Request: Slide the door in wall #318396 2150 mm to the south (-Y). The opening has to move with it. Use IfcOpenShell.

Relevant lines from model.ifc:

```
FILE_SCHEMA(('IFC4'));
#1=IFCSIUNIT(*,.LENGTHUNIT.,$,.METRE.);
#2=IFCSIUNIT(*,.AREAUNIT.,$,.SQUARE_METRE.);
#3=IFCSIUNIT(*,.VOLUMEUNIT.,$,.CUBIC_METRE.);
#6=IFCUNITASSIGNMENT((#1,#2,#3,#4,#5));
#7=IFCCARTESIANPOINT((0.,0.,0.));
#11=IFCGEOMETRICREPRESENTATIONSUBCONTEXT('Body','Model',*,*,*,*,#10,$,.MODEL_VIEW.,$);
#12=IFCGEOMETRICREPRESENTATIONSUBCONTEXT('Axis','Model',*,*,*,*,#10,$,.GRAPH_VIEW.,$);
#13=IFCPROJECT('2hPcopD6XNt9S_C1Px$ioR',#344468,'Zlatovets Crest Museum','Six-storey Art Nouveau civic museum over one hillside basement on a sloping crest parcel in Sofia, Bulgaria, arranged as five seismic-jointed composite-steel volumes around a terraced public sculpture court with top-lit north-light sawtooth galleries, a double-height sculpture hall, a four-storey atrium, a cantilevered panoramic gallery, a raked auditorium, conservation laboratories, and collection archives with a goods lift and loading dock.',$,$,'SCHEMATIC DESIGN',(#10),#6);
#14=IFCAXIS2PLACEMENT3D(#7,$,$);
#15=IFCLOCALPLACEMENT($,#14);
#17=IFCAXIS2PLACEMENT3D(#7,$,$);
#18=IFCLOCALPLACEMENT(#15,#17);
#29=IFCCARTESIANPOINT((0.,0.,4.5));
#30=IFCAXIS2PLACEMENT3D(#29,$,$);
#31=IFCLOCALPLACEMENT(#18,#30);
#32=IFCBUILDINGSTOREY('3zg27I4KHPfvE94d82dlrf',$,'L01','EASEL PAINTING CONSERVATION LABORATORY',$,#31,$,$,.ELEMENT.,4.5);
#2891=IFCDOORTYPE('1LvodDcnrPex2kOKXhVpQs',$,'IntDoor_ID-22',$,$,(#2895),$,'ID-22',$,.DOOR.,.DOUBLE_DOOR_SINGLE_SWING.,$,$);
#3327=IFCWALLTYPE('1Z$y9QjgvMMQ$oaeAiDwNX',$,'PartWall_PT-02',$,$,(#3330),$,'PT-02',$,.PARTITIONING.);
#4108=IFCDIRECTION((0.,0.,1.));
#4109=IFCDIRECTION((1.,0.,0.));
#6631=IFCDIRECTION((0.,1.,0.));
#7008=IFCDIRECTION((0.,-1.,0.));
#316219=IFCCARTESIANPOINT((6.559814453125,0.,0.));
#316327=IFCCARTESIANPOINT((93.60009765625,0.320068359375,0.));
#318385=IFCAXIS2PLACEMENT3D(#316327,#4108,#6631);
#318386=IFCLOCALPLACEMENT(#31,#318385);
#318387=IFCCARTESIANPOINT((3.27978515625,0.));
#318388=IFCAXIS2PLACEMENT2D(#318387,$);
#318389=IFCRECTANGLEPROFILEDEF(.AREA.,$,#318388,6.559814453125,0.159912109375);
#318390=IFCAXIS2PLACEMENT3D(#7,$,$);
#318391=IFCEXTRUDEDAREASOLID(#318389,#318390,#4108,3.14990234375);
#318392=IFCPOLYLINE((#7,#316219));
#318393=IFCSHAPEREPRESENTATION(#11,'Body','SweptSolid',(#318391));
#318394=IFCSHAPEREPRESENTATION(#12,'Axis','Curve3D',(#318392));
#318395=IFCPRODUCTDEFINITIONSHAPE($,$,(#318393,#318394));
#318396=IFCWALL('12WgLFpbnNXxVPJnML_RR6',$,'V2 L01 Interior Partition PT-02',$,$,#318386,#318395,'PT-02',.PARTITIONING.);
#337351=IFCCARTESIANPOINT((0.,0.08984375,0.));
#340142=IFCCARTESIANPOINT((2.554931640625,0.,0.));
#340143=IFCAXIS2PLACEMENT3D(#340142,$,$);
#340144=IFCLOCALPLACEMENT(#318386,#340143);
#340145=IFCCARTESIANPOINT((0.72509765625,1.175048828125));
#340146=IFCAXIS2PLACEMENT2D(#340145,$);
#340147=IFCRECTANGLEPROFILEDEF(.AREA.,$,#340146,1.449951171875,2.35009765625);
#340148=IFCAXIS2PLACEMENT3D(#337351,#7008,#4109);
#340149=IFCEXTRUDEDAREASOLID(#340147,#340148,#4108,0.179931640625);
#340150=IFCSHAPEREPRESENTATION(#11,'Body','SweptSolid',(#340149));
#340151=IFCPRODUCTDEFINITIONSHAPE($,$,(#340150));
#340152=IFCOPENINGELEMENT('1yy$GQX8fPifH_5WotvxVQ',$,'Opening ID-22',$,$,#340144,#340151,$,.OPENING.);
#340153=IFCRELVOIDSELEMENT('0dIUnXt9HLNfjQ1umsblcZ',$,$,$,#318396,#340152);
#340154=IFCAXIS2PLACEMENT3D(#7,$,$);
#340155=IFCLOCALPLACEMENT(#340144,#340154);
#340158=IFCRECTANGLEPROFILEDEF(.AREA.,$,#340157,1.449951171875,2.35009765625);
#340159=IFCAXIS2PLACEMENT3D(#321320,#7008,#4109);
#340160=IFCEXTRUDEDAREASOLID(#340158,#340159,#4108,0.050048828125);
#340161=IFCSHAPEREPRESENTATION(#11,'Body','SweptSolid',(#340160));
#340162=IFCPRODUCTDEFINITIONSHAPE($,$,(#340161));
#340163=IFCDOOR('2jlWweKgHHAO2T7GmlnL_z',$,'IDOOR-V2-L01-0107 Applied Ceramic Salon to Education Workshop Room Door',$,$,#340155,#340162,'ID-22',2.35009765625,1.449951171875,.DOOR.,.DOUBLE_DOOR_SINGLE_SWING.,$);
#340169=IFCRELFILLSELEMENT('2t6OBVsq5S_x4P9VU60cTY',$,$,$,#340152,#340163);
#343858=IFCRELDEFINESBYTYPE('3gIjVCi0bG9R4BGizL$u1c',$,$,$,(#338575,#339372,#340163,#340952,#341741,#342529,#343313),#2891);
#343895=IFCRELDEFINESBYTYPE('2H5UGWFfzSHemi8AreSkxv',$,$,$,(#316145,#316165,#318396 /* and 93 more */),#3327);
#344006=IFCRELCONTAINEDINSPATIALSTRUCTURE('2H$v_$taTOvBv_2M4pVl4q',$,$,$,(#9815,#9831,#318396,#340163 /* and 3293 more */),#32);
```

```python
import ifcopenshell
import ifcopenshell.api.geometry
import ifcopenshell.util.placement

model = ifcopenshell.open("model.ifc")

door = model.by_id(340163)
opening = door.FillsVoids[0].RelatingOpeningElement
wall = opening.VoidsElements[0].RelatingBuildingElement

wall_matrix = ifcopenshell.util.placement.get_local_placement(wall.ObjectPlacement)
shift = wall_matrix[:3, 0] * -2.15
before = ifcopenshell.util.placement.get_local_placement(door.ObjectPlacement)[:3, 3].copy()

# The door is placed relative to its opening, so it follows when the opening moves.
matrix = ifcopenshell.util.placement.get_local_placement(opening.ObjectPlacement)
matrix[:3, 3] += shift
ifcopenshell.api.geometry.edit_object_placement(
    model, product=opening, matrix=matrix, is_si=False, should_transform_children=True
)

after = ifcopenshell.util.placement.get_local_placement(door.ObjectPlacement)[:3, 3]
print("door moved by", (after - before).round(3) + 0.0)

model.write("model-out.ifc")
```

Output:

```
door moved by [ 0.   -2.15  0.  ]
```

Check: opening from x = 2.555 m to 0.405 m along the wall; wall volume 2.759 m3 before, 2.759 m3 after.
